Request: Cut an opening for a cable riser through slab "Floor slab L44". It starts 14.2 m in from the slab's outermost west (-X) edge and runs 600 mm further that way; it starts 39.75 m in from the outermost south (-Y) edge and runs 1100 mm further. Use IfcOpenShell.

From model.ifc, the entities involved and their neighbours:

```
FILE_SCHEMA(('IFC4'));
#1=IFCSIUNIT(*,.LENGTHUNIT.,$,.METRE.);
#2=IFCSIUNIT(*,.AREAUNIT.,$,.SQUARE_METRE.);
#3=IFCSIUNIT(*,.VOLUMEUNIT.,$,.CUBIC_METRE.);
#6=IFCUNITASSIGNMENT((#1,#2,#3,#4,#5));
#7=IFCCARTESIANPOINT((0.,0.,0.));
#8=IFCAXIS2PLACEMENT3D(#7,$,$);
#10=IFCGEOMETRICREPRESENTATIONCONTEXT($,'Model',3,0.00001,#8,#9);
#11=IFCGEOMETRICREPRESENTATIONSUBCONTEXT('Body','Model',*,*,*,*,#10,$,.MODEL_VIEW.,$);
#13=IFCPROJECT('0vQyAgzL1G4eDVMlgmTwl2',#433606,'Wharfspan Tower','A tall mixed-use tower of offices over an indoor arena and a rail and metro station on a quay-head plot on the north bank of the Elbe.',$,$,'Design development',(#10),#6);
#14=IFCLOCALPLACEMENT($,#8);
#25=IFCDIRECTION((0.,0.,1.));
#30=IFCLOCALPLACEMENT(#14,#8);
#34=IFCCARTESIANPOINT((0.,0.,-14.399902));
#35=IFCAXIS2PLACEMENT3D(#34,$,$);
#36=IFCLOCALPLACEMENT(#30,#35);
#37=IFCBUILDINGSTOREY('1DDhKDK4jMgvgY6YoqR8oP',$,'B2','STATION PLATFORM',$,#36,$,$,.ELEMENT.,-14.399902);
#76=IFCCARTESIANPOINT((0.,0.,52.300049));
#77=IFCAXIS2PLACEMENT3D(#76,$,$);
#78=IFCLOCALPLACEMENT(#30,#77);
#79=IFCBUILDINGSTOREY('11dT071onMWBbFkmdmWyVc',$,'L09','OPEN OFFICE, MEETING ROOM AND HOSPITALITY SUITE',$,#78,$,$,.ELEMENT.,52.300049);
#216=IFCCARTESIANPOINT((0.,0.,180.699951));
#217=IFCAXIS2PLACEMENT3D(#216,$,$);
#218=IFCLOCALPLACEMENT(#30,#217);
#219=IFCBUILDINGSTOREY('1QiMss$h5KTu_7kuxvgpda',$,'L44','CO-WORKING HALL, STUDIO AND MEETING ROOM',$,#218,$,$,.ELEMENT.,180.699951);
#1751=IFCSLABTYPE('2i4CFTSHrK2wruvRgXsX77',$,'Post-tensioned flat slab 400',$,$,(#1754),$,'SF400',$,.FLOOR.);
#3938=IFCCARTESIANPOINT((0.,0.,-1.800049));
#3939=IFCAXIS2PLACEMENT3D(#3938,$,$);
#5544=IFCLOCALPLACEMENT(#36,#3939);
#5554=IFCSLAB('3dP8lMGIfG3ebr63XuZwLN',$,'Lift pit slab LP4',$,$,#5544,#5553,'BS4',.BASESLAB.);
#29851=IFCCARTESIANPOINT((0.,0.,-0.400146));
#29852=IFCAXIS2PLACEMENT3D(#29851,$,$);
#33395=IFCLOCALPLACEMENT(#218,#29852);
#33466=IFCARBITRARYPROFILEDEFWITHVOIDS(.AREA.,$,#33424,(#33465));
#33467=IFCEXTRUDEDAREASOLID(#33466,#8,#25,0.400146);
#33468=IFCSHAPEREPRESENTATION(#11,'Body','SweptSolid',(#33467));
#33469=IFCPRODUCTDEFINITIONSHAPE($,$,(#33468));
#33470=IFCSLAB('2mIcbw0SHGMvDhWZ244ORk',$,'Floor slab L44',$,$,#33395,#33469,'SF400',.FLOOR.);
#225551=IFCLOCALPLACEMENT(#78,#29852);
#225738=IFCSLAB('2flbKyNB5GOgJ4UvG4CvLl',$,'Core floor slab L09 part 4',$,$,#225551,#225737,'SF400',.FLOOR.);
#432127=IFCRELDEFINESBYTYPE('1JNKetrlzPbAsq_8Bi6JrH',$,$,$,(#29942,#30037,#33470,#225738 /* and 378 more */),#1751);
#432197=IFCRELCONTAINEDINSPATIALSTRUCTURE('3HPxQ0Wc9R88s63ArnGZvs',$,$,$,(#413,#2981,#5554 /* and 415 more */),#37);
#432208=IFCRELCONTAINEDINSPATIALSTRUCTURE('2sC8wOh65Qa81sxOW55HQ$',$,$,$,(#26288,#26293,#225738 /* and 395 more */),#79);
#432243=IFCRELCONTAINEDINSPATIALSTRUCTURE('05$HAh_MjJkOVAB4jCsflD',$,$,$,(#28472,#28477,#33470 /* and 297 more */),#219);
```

```python
import numpy as np
import ifcopenshell
import ifcopenshell.api.feature
import ifcopenshell.api.geometry
import ifcopenshell.api.root
import ifcopenshell.geom
import ifcopenshell.util.placement
import ifcopenshell.util.representation
import ifcopenshell.util.shape
import ifcopenshell.util.unit

model = ifcopenshell.open("model.ifc")
unit_scale = ifcopenshell.util.unit.calculate_unit_scale(model)
settings = ifcopenshell.geom.settings()


def volume(element):
    """Net volume in cubic metres, openings subtracted."""
    shape = ifcopenshell.geom.create_shape(settings, element)
    return ifcopenshell.util.shape.get_volume(shape.geometry)


slab = model.by_guid("2mIcbw0SHGMvDhWZ244ORk")
before = volume(slab)

# Extent in the slab's own axes, in metres. The edges named are its -X and -Y sides.
slab_shape = ifcopenshell.geom.create_shape(settings, slab)
vertices = ifcopenshell.util.shape.get_vertices(slab_shape.geometry)
x_min, y_min, bottom = vertices.min(axis=0)
top = vertices[:, 2].max()

opening = ifcopenshell.api.root.create_entity(model, ifc_class="IfcOpeningElement", name="Cable riser opening", predefined_type="OPENING")
context = ifcopenshell.util.representation.get_context(model, "Model", "Body", "MODEL_VIEW")
width, depth = 0.6, 1.1
outline = [(0.0, 0.0), (width, 0.0), (width, depth), (0.0, depth), (0.0, 0.0)]
# Overshoot both faces by 50 mm so the cut is clean.
shape = ifcopenshell.api.geometry.add_slab_representation(
    model, context=context, depth=top - bottom + 0.1, polyline=outline
)
ifcopenshell.api.geometry.assign_representation(model, product=opening, representation=shape)

matrix = ifcopenshell.util.placement.get_local_placement(slab.ObjectPlacement)
matrix[:, 3] = matrix @ np.append(np.array([x_min + 14.2, y_min + 39.75, bottom - 0.05]) / unit_scale, 1.0)
ifcopenshell.api.geometry.edit_object_placement(model, product=opening, matrix=matrix, is_si=False)
ifcopenshell.api.feature.add_feature(model, feature=opening, element=slab)

after = volume(slab)

print(f"slab volume {before:.3f} -> {after:.3f} m3")

model.write("model_rev.ifc")
```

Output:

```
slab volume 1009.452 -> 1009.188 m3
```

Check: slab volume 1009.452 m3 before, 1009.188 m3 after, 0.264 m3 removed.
